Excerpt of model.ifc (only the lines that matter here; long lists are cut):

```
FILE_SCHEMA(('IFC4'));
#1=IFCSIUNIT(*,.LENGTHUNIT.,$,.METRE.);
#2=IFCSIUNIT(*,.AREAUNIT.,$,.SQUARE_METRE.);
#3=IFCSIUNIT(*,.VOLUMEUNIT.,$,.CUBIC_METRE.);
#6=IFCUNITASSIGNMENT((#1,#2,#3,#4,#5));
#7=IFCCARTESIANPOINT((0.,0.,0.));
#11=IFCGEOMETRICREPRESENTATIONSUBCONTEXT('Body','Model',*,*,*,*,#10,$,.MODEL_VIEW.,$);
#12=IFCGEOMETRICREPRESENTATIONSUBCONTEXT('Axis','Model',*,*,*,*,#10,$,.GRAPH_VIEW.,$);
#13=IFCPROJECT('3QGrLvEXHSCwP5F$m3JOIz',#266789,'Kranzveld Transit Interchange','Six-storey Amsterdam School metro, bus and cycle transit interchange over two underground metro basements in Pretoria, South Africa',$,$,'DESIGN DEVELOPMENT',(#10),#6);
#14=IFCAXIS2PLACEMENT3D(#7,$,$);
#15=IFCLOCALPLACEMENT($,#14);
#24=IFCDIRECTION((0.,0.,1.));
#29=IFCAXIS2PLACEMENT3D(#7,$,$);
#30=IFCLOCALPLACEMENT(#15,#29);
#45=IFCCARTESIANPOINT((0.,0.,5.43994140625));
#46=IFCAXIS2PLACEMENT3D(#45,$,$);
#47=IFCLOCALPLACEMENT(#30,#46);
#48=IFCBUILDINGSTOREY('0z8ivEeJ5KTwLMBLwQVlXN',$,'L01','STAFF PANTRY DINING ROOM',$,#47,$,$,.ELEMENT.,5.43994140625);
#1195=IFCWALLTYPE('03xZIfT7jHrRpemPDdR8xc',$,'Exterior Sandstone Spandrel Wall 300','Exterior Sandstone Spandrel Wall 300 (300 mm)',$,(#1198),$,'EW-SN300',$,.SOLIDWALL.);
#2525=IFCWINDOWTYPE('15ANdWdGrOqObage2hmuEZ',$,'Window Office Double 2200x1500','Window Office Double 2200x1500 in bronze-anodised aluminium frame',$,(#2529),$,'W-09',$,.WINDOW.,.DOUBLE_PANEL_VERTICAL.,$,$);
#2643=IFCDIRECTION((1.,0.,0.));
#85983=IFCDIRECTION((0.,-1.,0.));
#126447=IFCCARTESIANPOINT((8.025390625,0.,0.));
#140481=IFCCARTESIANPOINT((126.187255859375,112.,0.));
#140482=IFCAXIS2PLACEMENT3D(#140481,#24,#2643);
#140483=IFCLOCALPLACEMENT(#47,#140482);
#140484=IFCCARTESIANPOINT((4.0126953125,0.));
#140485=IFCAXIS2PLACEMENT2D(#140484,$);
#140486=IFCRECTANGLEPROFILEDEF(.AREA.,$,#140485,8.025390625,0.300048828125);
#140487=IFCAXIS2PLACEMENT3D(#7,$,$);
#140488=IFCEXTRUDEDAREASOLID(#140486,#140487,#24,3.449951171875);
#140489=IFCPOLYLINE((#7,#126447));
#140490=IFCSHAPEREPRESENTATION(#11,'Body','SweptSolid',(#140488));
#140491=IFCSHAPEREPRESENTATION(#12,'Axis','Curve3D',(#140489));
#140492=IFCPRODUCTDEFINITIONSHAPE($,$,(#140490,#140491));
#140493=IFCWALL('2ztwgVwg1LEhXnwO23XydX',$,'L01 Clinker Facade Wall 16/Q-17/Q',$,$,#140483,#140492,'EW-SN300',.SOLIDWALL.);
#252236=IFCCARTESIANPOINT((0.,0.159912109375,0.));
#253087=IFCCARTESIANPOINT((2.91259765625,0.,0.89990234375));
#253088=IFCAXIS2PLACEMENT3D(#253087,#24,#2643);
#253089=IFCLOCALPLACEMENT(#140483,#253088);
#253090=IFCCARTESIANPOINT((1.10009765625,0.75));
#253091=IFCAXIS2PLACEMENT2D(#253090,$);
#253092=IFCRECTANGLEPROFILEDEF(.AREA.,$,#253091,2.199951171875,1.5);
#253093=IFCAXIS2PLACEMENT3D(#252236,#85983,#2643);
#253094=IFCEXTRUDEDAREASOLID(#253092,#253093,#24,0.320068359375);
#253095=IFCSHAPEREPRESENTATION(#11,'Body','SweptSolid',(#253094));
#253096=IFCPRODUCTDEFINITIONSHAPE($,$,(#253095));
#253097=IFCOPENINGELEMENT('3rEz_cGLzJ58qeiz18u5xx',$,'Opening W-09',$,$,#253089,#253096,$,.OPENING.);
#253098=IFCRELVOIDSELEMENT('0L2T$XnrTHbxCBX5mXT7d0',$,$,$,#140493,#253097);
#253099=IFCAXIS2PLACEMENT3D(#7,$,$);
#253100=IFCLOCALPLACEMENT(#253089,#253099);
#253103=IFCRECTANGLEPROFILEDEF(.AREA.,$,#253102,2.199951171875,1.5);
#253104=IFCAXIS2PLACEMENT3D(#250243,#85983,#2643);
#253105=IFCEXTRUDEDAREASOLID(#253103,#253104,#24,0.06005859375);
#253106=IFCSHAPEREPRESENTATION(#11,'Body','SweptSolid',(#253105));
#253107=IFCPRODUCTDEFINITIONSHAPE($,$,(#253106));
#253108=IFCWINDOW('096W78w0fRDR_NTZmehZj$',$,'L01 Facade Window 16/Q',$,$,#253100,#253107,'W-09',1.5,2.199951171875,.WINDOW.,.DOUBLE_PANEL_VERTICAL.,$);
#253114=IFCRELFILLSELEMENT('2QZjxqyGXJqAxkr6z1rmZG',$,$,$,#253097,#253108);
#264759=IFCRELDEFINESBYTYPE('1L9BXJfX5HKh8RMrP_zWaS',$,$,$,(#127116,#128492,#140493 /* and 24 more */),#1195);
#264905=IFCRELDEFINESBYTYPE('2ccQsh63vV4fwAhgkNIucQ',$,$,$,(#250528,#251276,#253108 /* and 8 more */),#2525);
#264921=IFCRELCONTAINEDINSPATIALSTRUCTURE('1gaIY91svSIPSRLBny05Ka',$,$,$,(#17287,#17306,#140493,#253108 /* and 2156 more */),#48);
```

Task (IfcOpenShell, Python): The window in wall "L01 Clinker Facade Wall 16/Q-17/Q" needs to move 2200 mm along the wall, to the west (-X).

```python
import ifcopenshell
import ifcopenshell.api.geometry
import ifcopenshell.util.placement
import ifcopenshell.util.unit

model = ifcopenshell.open("model.ifc")
unit_scale = ifcopenshell.util.unit.calculate_unit_scale(model)

window = model.by_guid("096W78w0fRDR_NTZmehZj$")
opening = window.FillsVoids[0].RelatingOpeningElement
wall = opening.VoidsElements[0].RelatingBuildingElement

wall_matrix = ifcopenshell.util.placement.get_local_placement(wall.ObjectPlacement)
shift = wall_matrix[:3, 0] * -2.2 / unit_scale
before = ifcopenshell.util.placement.get_local_placement(window.ObjectPlacement)[:3, 3].copy()

# The window is placed relative to its opening, so it follows when the opening moves.
matrix = ifcopenshell.util.placement.get_local_placement(opening.ObjectPlacement)
matrix[:3, 3] += shift
ifcopenshell.api.geometry.edit_object_placement(
    model, product=opening, matrix=matrix, is_si=False, should_transform_children=True
)

after = ifcopenshell.util.placement.get_local_placement(window.ObjectPlacement)[:3, 3]
print("window moved by", (after - before).round(3) + 0.0)

model.write("model_v2.ifc")
```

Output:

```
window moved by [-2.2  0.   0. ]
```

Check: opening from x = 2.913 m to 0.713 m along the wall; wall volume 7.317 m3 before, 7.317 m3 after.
